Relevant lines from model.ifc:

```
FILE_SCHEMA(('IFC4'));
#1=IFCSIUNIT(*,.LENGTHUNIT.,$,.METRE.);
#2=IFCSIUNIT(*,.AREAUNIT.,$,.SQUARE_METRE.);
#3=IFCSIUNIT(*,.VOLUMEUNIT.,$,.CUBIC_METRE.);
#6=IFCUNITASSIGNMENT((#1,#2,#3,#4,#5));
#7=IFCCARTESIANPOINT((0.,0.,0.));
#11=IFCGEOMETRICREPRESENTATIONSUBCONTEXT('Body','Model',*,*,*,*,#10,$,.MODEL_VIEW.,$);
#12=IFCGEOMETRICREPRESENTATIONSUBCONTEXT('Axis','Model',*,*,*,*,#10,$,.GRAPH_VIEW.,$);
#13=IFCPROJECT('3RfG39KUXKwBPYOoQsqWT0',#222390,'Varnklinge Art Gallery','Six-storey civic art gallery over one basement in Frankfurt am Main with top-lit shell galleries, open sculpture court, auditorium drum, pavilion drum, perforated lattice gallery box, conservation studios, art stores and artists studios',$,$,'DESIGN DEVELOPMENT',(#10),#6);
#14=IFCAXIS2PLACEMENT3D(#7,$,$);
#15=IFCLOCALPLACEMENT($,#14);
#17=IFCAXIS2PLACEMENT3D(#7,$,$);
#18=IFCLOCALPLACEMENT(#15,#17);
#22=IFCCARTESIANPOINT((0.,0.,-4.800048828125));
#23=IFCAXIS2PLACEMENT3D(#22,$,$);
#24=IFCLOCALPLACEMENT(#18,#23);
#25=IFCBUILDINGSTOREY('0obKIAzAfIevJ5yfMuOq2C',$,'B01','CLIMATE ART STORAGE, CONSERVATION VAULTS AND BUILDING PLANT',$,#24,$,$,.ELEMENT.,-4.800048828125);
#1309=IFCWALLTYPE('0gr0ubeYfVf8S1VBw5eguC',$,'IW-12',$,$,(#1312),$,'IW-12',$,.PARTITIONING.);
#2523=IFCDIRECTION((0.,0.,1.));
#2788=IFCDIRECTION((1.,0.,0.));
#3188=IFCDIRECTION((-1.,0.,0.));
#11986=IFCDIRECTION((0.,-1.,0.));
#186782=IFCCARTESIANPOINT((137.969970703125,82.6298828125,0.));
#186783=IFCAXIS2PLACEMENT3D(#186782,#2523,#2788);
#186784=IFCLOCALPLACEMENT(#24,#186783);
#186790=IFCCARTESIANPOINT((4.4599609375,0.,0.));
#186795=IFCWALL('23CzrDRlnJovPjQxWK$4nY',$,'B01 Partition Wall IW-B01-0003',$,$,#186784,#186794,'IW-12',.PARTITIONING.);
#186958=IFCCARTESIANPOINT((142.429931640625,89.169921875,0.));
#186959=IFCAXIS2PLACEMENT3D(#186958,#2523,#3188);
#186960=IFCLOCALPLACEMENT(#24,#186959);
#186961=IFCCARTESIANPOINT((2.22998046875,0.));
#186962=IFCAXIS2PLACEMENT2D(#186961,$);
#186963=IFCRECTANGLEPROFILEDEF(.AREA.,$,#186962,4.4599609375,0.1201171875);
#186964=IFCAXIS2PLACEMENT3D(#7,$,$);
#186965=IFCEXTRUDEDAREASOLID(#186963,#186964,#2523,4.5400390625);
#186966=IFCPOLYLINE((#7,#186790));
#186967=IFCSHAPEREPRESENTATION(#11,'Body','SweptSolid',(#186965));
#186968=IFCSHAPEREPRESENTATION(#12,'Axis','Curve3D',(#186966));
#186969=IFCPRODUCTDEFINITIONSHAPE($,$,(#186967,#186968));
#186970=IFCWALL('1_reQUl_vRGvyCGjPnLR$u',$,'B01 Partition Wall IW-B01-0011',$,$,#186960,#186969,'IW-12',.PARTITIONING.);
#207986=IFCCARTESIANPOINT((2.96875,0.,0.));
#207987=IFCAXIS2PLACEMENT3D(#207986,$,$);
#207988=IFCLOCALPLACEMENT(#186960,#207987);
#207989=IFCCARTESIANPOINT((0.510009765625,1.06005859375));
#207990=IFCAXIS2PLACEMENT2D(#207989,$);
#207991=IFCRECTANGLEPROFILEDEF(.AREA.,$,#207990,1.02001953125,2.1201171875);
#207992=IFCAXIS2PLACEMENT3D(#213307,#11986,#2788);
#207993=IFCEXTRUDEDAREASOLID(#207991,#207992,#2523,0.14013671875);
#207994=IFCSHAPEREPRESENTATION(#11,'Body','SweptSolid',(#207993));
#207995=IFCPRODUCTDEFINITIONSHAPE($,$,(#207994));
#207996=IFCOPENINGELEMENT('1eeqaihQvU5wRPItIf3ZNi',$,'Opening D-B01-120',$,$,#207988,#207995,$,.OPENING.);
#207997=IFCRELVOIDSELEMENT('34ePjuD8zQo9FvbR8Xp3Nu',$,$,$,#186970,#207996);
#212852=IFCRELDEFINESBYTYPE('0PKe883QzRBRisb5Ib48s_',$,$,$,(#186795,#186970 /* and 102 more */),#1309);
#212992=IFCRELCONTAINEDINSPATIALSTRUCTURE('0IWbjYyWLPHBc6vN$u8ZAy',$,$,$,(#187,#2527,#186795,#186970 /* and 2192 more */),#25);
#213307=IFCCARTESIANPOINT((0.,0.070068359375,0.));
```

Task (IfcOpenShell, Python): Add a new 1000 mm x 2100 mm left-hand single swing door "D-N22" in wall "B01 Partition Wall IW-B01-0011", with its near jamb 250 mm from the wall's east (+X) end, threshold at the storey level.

```python
import numpy as np
import ifcopenshell
import ifcopenshell.api.feature
import ifcopenshell.api.geometry
import ifcopenshell.api.root
import ifcopenshell.api.spatial
import ifcopenshell.geom
import ifcopenshell.util.element
import ifcopenshell.util.placement
import ifcopenshell.util.representation
import ifcopenshell.util.shape
import ifcopenshell.util.unit

model = ifcopenshell.open("model.ifc")
unit_scale = ifcopenshell.util.unit.calculate_unit_scale(model)
settings = ifcopenshell.geom.settings()


def volume(element):
    """Net volume in cubic metres, openings subtracted."""
    shape = ifcopenshell.geom.create_shape(settings, element)
    return ifcopenshell.util.shape.get_volume(shape.geometry)


wall = model.by_guid("1_reQUl_vRGvyCGjPnLR$u")
storey = ifcopenshell.util.element.get_container(wall, ifc_class="IfcBuildingStorey")
context = ifcopenshell.util.representation.get_context(model, "Model", "Body", "MODEL_VIEW")
before = volume(wall)

width, height, from_end, sill = 1, 2.1, 0.25, 0.0  # metres

# The wall runs along its own X axis, and the end named is its -X end.
wall_shape = ifcopenshell.geom.create_shape(settings, wall)
x, y, z = ifcopenshell.util.shape.get_vertices(wall_shape.geometry).T
start = x.min() + from_end
face, thickness = float(y.min()), float(y.max() - y.min())
wall_matrix = ifcopenshell.util.placement.get_local_placement(wall.ObjectPlacement)
level = ifcopenshell.util.placement.get_local_placement(storey.ObjectPlacement)[2, 3]


def in_wall(x, y):
    """Placement at x, y metres in the wall's axes, at sill height."""
    matrix = wall_matrix.copy()
    matrix[:, 3] = wall_matrix @ np.array([x / unit_scale, y / unit_scale, 0.0, 1.0])
    matrix[2, 3] = level + sill / unit_scale
    return matrix


# Opening: a box that overshoots both wall faces by 50 mm.
opening = ifcopenshell.api.root.create_entity(model, ifc_class="IfcOpeningElement", predefined_type="OPENING")
box = ifcopenshell.api.geometry.add_wall_representation(
    model, context=context, length=width, height=height, thickness=thickness + 0.1
)
ifcopenshell.api.geometry.assign_representation(model, product=opening, representation=box)
ifcopenshell.api.geometry.edit_object_placement(model, product=opening, matrix=in_wall(start, face - 0.05), is_si=False)
ifcopenshell.api.feature.add_feature(model, feature=opening, element=wall)

door = ifcopenshell.api.root.create_entity(model, ifc_class="IfcDoor", name="D-N22", predefined_type="DOOR")
door.OverallWidth, door.OverallHeight = width / unit_scale, height / unit_scale
door.OperationType = "SINGLE_SWING_LEFT"
body = ifcopenshell.api.geometry.add_door_representation(
    model,
    context=context,
    overall_width=door.OverallWidth,
    overall_height=door.OverallHeight,
    operation_type="SINGLE_SWING_LEFT",
    lining_properties={"LiningDepth": thickness / unit_scale, "ThresholdDepth": thickness / unit_scale},
)
ifcopenshell.api.geometry.assign_representation(model, product=door, representation=body)
ifcopenshell.api.spatial.assign_container(model, products=[door], relating_structure=storey)
ifcopenshell.api.feature.add_filling(model, opening=opening, element=door)

# The lining spans the wall, so the door starts at the wall face.
ifcopenshell.api.geometry.edit_object_placement(model, product=door, matrix=in_wall(start, face), is_si=False)

after = volume(wall)

print(f"wall volume {before:.3f} -> {after:.3f} m3")

model.write("model-out.ifc")
```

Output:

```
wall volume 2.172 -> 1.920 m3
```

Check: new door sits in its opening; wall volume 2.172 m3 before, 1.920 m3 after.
